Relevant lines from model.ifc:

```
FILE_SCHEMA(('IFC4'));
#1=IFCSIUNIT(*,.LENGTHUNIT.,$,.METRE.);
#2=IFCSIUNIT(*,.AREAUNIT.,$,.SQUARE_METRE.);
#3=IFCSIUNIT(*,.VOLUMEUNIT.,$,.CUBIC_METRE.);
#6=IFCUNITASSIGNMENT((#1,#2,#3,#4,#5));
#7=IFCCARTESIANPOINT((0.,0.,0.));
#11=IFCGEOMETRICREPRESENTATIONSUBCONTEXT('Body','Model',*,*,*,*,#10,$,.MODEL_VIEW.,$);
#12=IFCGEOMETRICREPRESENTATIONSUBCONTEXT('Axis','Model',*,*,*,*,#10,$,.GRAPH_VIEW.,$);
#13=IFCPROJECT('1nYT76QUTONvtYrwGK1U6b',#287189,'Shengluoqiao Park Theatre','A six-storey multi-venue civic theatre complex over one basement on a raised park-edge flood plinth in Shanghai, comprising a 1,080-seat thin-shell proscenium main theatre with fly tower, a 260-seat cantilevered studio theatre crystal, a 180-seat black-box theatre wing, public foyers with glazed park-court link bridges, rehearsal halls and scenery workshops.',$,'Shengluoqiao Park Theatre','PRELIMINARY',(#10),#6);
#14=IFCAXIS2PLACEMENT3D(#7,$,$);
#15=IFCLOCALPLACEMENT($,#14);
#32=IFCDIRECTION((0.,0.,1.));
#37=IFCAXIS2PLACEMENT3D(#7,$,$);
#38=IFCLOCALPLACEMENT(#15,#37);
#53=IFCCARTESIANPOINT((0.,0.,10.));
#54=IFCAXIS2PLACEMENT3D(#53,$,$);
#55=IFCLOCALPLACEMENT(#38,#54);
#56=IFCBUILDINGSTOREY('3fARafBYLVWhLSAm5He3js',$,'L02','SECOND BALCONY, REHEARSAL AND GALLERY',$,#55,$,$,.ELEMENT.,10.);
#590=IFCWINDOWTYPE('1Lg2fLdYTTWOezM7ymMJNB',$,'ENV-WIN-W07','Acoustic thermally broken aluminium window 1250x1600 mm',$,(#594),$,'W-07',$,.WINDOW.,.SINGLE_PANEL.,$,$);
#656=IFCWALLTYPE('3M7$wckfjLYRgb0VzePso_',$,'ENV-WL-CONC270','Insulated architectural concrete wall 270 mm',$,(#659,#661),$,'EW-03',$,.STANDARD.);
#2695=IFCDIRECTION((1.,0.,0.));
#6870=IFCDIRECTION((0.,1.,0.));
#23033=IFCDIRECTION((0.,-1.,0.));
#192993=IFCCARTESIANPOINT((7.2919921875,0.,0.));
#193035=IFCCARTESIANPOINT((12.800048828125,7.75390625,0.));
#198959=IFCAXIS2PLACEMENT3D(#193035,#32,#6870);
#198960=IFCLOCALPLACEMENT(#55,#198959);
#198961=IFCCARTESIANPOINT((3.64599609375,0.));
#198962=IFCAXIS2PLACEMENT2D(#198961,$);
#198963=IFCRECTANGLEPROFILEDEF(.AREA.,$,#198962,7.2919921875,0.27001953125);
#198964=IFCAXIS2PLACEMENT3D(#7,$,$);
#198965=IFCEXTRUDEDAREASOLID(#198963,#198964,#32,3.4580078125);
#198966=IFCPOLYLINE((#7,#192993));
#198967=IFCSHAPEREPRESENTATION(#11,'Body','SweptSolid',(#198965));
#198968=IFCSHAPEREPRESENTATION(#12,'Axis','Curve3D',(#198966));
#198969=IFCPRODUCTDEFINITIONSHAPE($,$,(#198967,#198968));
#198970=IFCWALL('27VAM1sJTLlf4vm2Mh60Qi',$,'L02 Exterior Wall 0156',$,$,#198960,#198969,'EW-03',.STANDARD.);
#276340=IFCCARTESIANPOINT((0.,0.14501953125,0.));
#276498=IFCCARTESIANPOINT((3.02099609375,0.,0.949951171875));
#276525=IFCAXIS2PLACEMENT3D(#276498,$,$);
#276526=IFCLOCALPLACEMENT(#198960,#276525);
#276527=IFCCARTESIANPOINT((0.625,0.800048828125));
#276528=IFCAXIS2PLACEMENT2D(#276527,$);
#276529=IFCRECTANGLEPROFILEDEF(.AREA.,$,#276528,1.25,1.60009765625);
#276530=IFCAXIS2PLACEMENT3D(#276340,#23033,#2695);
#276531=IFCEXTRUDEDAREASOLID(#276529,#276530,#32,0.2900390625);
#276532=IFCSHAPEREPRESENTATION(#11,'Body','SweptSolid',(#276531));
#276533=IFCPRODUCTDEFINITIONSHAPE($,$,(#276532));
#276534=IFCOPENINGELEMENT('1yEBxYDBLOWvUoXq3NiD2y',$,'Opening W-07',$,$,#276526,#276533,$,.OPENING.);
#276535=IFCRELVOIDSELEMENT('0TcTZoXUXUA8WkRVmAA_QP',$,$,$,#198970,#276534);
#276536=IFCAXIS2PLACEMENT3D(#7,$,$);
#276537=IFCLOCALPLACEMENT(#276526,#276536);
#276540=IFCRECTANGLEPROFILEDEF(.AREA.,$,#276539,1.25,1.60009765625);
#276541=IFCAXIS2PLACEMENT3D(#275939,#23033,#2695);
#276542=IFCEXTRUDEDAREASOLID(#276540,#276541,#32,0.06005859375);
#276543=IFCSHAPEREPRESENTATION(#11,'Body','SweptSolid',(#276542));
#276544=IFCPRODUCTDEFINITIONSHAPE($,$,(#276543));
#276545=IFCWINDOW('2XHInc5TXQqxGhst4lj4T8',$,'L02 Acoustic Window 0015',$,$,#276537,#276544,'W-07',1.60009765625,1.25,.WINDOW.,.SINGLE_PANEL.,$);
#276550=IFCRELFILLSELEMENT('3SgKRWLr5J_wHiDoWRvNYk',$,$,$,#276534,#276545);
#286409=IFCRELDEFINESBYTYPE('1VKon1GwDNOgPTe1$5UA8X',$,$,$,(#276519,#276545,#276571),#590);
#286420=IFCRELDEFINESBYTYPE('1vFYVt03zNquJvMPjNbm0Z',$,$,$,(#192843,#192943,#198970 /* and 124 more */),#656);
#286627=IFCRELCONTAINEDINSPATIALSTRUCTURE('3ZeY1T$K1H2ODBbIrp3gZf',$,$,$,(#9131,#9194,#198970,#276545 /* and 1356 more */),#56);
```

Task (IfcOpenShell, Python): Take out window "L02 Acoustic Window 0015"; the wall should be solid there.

```python
import ifcopenshell
import ifcopenshell.api.feature
import ifcopenshell.api.root
import ifcopenshell.geom
import ifcopenshell.util.shape

model = ifcopenshell.open("model.ifc")
settings = ifcopenshell.geom.settings()


def volume(element):
    """Net volume in cubic metres, openings subtracted."""
    shape = ifcopenshell.geom.create_shape(settings, element)
    return ifcopenshell.util.shape.get_volume(shape.geometry)


window = model.by_id(276545)
opening = window.FillsVoids[0].RelatingOpeningElement
wall = opening.VoidsElements[0].RelatingBuildingElement
before = volume(wall)

ifcopenshell.api.root.remove_product(model, product=window)
ifcopenshell.api.feature.remove_feature(model, feature=opening)

after = volume(wall)

print(f"wall volume {before:.3f} -> {after:.3f} m3")

model.write("model_v2.ifc")
```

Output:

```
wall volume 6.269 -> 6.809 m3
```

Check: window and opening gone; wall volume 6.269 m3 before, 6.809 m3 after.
